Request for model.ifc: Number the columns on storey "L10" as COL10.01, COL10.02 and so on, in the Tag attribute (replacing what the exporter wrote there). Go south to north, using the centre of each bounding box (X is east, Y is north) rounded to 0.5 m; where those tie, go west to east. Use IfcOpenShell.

First a look at what the model holds.

```python
import ifcopenshell
import ifcopenshell.util.element
import ifcopenshell.util.placement

model = ifcopenshell.open("model.ifc")
print(model.schema)
storey = next(s for s in model.by_type("IfcBuildingStorey") if s.Name == "L10")
columns = [e for e in ifcopenshell.util.element.get_decomposition(storey) if e.is_a("IfcColumn")]
for e in sorted(columns, key=lambda e: e.id()):
    origin = ifcopenshell.util.placement.get_local_placement(e.ObjectPlacement)[:3, 3]
    print(e.id(), e.Tag, e.Name, origin.round(2) + 0.0, sep=" | ")
```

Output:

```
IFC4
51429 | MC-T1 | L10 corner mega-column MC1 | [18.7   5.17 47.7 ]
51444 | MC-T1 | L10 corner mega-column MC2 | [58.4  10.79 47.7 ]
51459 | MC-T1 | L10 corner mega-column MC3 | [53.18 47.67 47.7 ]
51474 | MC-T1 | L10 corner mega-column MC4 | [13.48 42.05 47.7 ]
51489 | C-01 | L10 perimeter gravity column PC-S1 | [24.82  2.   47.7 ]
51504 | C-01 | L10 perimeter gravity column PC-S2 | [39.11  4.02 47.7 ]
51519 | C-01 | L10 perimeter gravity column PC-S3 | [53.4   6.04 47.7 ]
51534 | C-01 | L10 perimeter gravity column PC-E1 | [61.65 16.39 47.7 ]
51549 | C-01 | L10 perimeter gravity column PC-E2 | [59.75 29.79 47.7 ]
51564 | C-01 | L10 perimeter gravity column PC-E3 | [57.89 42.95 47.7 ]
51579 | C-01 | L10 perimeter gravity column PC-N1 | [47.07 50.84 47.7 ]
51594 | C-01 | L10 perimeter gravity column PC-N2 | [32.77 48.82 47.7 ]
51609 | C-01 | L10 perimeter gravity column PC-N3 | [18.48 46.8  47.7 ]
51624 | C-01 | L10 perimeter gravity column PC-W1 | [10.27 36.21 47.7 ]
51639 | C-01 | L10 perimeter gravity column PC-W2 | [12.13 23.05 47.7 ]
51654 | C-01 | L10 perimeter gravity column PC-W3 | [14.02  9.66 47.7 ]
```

```python
import ifcopenshell
import ifcopenshell.geom
import ifcopenshell.util.element
import ifcopenshell.util.shape

model = ifcopenshell.open("model.ifc")
settings = ifcopenshell.geom.settings()
settings.set("use-world-coords", True)


def centre(element):
    shape = ifcopenshell.geom.create_shape(settings, element)
    return ifcopenshell.util.shape.get_bbox_centroid(shape.geometry)


storey = next(s for s in model.by_type("IfcBuildingStorey") if s.Name == "L10")
columns = [e for e in ifcopenshell.util.element.get_decomposition(storey) if e.is_a("IfcColumn")]

# Insertion points can sit at a corner or the storey origin, so sort by the geometry (in metres).
centres = {e: centre(e) for e in columns}
columns.sort(key=lambda e: (round(centres[e][1] / 0.5), centres[e][0]))

for i, e in enumerate(columns, start=1):
    number = f"COL10.{i:02d}"
    e.Tag = number
    print(e.id(), number)

model.write("model_rev.ifc")
```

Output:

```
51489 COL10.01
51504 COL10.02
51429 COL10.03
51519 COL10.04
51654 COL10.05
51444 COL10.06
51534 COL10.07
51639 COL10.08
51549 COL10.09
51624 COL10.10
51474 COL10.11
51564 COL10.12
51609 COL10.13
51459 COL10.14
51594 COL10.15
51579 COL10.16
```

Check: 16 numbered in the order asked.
